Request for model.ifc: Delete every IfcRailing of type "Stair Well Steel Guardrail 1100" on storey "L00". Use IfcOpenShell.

First a look at what the model holds.

```python
import ifcopenshell
import ifcopenshell.util.element

model = ifcopenshell.open("model.ifc")
print(model.schema)
storey = next(s for s in model.by_type("IfcBuildingStorey") if s.Name == "L00")
railings = [e for e in ifcopenshell.util.element.get_decomposition(storey) if e.is_a("IfcRailing")]
seen = {}
for e in railings:
    element_type = ifcopenshell.util.element.get_type(e)
    name = element_type.Name if element_type not in (None, e) else None
    seen[name] = seen.get(name, 0) + 1
for name, count in sorted(seen.items(), key=str):
    print(count, "x", name)
```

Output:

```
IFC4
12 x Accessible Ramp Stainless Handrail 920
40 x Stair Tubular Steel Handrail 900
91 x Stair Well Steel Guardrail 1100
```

```python
import ifcopenshell
import ifcopenshell.api.root
import ifcopenshell.util.element

model = ifcopenshell.open("model.ifc")

storey = next(s for s in model.by_type("IfcBuildingStorey") if s.Name == "L00")
railings = [e for e in ifcopenshell.util.element.get_decomposition(storey) if e.is_a("IfcRailing")]
targets = [e for e in railings if (t := ifcopenshell.util.element.get_type(e)) not in (None, e) and t.Name == "Stair Well Steel Guardrail 1100"]

for e in targets:
    ifcopenshell.api.root.remove_product(model, product=e)
print(len(targets), "removed")

model.write("model_edited.ifc")
```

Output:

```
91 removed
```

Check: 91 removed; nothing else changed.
